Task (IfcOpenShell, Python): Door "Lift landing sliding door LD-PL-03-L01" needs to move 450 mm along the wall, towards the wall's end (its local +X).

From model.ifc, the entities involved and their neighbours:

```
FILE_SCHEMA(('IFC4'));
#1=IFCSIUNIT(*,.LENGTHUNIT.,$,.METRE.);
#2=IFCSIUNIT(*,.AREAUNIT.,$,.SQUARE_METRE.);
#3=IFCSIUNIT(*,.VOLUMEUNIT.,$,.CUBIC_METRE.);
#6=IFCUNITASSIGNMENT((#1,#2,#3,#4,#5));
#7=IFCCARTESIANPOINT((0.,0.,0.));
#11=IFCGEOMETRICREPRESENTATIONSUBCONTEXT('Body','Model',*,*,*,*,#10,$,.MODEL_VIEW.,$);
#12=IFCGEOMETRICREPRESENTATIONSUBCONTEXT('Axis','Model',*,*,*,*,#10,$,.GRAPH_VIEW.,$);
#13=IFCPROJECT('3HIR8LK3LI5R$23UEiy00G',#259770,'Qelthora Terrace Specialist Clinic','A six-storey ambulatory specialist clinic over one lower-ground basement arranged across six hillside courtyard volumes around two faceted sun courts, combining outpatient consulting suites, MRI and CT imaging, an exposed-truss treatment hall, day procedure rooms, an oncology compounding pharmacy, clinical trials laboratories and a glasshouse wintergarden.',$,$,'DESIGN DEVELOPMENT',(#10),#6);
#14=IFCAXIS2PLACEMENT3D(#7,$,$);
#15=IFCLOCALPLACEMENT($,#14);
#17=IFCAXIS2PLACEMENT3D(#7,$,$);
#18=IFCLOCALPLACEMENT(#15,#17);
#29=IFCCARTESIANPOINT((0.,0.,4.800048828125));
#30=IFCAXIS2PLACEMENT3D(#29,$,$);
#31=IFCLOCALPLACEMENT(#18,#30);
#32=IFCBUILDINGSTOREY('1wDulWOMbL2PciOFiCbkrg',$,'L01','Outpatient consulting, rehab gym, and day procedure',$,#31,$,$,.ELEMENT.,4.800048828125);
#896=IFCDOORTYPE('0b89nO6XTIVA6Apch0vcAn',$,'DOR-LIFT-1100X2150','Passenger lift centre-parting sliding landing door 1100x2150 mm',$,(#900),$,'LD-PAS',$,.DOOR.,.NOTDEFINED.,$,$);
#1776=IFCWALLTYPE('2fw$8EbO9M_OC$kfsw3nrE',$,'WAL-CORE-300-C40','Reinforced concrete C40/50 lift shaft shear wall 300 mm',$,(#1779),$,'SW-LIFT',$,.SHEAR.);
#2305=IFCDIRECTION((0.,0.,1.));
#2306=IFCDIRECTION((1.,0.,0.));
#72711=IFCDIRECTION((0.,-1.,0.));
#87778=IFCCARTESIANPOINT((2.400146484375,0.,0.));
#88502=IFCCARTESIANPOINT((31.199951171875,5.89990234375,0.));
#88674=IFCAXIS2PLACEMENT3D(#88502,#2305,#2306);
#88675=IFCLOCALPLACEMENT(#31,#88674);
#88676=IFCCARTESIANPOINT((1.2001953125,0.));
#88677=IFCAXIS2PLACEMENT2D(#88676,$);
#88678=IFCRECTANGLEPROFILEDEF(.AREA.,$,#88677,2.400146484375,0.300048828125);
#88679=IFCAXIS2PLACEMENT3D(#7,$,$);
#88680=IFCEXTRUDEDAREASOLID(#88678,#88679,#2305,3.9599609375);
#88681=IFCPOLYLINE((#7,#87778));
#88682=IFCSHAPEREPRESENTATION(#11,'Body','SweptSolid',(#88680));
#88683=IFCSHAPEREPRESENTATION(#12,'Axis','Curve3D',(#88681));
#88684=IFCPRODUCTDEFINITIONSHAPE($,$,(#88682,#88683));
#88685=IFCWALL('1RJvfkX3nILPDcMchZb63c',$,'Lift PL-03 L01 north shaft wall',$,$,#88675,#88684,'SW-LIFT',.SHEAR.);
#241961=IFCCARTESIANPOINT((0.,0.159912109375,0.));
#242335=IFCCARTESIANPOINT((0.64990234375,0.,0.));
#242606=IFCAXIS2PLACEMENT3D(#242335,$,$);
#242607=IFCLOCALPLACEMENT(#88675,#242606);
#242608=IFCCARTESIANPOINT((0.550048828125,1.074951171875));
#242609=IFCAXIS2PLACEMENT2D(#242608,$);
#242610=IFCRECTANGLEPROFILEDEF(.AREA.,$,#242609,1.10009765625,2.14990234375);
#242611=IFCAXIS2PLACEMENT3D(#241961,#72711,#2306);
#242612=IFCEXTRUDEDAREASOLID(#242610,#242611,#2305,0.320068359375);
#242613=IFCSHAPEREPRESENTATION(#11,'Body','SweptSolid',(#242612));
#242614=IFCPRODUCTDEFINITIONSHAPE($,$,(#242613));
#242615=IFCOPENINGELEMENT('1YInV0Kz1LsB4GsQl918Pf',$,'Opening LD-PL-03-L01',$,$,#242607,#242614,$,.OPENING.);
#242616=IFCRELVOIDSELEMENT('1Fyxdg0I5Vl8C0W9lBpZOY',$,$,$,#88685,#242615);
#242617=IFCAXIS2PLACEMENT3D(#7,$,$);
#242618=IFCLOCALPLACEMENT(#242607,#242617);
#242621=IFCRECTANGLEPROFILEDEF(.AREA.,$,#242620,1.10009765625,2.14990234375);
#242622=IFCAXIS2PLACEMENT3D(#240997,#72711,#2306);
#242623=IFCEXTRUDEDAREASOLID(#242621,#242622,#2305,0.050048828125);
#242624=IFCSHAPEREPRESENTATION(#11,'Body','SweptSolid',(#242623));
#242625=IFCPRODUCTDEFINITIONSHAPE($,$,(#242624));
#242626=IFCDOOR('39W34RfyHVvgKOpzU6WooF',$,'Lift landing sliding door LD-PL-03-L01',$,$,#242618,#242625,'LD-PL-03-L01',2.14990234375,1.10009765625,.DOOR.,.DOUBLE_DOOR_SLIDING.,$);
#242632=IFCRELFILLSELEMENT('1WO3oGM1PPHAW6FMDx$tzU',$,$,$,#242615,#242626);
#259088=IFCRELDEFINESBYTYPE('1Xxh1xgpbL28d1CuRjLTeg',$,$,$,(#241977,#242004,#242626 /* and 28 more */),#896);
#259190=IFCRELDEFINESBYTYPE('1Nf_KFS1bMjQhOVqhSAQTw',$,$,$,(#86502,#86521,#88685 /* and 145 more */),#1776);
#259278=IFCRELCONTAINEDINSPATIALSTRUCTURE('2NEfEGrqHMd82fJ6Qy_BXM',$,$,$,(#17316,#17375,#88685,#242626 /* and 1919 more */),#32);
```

```python
import ifcopenshell
import ifcopenshell.api.geometry
import ifcopenshell.util.placement

model = ifcopenshell.open("model.ifc")

door = model.by_guid("39W34RfyHVvgKOpzU6WooF")
opening = door.FillsVoids[0].RelatingOpeningElement
wall = opening.VoidsElements[0].RelatingBuildingElement

wall_matrix = ifcopenshell.util.placement.get_local_placement(wall.ObjectPlacement)
shift = wall_matrix[:3, 0] * 0.45
before = ifcopenshell.util.placement.get_local_placement(door.ObjectPlacement)[:3, 3].copy()

# The door is placed relative to its opening, so it follows when the opening moves.
matrix = ifcopenshell.util.placement.get_local_placement(opening.ObjectPlacement)
matrix[:3, 3] += shift
ifcopenshell.api.geometry.edit_object_placement(
    model, product=opening, matrix=matrix, is_si=False, should_transform_children=True
)

after = ifcopenshell.util.placement.get_local_placement(door.ObjectPlacement)[:3, 3]
print("door moved by", (after - before).round(3) + 0.0)

model.write("model-out.ifc")
```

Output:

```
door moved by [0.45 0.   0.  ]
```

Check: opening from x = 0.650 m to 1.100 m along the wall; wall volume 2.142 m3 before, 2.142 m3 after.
